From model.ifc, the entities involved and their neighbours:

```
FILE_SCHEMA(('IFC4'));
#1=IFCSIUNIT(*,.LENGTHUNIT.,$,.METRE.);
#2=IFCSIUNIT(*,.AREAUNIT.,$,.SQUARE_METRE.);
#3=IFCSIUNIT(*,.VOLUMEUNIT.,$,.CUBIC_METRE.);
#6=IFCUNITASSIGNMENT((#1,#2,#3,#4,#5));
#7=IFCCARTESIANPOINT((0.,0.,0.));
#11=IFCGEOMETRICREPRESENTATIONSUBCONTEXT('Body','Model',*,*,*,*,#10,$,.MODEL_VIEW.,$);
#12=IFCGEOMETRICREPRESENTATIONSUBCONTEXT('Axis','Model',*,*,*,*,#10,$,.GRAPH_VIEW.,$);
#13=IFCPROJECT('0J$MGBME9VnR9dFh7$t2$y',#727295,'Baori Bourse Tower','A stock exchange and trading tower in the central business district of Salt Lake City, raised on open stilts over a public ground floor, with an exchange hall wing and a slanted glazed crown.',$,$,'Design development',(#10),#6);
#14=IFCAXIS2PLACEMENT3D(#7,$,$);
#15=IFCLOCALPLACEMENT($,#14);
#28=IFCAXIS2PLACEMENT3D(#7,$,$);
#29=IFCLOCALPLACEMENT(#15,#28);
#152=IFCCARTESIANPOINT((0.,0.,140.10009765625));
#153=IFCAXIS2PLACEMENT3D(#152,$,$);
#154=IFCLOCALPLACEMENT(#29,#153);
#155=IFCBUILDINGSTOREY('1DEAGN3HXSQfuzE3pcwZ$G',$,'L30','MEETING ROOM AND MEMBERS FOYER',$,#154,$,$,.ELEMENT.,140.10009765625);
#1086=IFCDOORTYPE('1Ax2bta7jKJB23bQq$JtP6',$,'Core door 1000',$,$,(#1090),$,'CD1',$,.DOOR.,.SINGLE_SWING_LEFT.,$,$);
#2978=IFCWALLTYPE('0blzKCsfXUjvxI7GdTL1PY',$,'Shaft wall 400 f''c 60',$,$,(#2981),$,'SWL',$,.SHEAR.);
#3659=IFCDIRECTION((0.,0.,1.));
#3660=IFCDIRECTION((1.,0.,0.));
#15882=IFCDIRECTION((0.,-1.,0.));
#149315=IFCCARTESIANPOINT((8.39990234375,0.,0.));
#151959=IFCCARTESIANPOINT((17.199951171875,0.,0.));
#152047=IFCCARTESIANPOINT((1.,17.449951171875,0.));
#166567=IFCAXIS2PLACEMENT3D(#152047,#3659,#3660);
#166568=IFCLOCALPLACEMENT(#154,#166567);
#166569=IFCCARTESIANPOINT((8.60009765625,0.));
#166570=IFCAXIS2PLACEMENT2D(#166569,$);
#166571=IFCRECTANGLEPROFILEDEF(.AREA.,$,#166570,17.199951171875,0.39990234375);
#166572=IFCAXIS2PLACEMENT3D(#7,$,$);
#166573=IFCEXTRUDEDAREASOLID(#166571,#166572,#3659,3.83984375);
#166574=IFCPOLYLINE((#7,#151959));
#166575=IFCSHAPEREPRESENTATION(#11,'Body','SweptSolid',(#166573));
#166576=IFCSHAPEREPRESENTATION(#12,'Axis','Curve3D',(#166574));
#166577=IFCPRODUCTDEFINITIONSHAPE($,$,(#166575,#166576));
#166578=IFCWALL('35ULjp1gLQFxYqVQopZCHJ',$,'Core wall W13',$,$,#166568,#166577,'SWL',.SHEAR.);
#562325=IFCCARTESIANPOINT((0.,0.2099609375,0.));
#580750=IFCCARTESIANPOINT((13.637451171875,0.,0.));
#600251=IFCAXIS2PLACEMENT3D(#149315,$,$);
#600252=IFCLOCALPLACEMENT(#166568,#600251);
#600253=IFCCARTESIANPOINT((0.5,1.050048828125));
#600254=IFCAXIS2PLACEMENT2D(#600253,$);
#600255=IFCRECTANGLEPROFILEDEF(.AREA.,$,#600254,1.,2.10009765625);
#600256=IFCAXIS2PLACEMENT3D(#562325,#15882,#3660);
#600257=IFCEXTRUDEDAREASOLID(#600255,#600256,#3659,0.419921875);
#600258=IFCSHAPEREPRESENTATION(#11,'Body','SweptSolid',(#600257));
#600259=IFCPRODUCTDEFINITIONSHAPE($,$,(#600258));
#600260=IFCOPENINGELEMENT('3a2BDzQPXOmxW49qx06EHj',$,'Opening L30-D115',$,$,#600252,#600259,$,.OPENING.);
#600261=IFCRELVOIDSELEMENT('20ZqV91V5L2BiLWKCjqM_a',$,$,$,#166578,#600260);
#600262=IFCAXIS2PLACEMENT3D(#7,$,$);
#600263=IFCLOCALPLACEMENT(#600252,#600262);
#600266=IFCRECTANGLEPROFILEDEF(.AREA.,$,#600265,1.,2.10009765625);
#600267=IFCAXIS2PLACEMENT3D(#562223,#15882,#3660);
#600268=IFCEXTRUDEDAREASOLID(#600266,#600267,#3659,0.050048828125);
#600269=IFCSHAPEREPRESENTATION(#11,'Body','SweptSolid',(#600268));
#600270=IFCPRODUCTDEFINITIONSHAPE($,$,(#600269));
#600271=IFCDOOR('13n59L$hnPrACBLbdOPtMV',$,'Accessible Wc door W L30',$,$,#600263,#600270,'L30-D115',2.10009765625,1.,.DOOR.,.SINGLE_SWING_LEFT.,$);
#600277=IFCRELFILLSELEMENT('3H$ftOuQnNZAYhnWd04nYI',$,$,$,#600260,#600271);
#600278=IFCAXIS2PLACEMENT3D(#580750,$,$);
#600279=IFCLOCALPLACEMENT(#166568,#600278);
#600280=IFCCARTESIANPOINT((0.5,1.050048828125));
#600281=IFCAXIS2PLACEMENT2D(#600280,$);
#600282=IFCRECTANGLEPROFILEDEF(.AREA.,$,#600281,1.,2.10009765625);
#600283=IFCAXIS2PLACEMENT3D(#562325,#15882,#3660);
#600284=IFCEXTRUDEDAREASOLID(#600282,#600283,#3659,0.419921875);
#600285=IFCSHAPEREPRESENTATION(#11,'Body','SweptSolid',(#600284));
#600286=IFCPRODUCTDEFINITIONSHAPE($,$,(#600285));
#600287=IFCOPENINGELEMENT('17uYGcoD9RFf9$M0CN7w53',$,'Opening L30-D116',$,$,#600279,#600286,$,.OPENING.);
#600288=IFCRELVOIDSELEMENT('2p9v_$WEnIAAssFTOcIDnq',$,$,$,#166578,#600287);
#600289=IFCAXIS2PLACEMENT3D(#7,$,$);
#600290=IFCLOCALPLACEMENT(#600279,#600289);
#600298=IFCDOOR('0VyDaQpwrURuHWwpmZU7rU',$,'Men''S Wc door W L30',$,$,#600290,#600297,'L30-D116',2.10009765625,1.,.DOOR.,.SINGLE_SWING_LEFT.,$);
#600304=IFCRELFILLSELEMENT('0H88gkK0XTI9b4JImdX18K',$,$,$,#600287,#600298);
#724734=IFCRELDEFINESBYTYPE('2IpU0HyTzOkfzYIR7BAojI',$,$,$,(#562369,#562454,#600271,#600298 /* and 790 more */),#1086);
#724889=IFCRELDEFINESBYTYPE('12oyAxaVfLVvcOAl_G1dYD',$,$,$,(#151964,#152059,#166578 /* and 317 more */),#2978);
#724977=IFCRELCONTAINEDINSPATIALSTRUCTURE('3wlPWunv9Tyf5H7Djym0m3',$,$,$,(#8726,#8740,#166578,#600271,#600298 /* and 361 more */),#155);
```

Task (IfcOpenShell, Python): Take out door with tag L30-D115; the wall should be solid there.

```python
import ifcopenshell
import ifcopenshell.api.feature
import ifcopenshell.api.root
import ifcopenshell.geom
import ifcopenshell.util.shape

model = ifcopenshell.open("model.ifc")
settings = ifcopenshell.geom.settings()


def volume(element):
    """Net volume in cubic metres, openings subtracted."""
    shape = ifcopenshell.geom.create_shape(settings, element)
    return ifcopenshell.util.shape.get_volume(shape.geometry)


door = model.by_guid("13n59L$hnPrACBLbdOPtMV")
opening = door.FillsVoids[0].RelatingOpeningElement
wall = opening.VoidsElements[0].RelatingBuildingElement
before = volume(wall)

ifcopenshell.api.root.remove_product(model, product=door)
ifcopenshell.api.feature.remove_feature(model, feature=opening)

after = volume(wall)

print(f"wall volume {before:.3f} -> {after:.3f} m3")

model.write("model_edited.ifc")
```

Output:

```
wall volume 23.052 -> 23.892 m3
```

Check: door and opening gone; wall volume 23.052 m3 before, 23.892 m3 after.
